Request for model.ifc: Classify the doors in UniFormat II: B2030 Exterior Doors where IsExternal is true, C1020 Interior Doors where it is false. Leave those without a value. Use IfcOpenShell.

First a look at what the model holds.

```python
import ifcopenshell
import ifcopenshell.util.element

model = ifcopenshell.open("model.ifc")
print(model.schema)
print("classifications:", [c.Name for c in model.by_type("IfcClassification")])
values = [ifcopenshell.util.element.get_pset(e, "Pset_DoorCommon", "IsExternal") for e in model.by_type("IfcDoor")]
for value in (True, False, None):
    print("IsExternal", value, values.count(value))
```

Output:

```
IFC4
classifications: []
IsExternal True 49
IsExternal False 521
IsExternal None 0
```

```python
import ifcopenshell
import ifcopenshell.api.classification
import ifcopenshell.util.element

model = ifcopenshell.open("model.ifc")

system = ifcopenshell.api.classification.add_classification(model, classification="UniFormat II")

doors = model.by_type("IfcDoor")
external = {e: ifcopenshell.util.element.get_pset(e, "Pset_DoorCommon", "IsExternal") for e in doors}
for flag, code, name in ((True, "B2030", "Exterior Doors"), (False, "C1020", "Interior Doors")):
    products = [e for e in doors if external[e] is flag]
    ifcopenshell.api.classification.add_reference(
        model, products=products, classification=system, identification=code, name=name
    )
    print(code, len(products))

model.write("model-out.ifc")
```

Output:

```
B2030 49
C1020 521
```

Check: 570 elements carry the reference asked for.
